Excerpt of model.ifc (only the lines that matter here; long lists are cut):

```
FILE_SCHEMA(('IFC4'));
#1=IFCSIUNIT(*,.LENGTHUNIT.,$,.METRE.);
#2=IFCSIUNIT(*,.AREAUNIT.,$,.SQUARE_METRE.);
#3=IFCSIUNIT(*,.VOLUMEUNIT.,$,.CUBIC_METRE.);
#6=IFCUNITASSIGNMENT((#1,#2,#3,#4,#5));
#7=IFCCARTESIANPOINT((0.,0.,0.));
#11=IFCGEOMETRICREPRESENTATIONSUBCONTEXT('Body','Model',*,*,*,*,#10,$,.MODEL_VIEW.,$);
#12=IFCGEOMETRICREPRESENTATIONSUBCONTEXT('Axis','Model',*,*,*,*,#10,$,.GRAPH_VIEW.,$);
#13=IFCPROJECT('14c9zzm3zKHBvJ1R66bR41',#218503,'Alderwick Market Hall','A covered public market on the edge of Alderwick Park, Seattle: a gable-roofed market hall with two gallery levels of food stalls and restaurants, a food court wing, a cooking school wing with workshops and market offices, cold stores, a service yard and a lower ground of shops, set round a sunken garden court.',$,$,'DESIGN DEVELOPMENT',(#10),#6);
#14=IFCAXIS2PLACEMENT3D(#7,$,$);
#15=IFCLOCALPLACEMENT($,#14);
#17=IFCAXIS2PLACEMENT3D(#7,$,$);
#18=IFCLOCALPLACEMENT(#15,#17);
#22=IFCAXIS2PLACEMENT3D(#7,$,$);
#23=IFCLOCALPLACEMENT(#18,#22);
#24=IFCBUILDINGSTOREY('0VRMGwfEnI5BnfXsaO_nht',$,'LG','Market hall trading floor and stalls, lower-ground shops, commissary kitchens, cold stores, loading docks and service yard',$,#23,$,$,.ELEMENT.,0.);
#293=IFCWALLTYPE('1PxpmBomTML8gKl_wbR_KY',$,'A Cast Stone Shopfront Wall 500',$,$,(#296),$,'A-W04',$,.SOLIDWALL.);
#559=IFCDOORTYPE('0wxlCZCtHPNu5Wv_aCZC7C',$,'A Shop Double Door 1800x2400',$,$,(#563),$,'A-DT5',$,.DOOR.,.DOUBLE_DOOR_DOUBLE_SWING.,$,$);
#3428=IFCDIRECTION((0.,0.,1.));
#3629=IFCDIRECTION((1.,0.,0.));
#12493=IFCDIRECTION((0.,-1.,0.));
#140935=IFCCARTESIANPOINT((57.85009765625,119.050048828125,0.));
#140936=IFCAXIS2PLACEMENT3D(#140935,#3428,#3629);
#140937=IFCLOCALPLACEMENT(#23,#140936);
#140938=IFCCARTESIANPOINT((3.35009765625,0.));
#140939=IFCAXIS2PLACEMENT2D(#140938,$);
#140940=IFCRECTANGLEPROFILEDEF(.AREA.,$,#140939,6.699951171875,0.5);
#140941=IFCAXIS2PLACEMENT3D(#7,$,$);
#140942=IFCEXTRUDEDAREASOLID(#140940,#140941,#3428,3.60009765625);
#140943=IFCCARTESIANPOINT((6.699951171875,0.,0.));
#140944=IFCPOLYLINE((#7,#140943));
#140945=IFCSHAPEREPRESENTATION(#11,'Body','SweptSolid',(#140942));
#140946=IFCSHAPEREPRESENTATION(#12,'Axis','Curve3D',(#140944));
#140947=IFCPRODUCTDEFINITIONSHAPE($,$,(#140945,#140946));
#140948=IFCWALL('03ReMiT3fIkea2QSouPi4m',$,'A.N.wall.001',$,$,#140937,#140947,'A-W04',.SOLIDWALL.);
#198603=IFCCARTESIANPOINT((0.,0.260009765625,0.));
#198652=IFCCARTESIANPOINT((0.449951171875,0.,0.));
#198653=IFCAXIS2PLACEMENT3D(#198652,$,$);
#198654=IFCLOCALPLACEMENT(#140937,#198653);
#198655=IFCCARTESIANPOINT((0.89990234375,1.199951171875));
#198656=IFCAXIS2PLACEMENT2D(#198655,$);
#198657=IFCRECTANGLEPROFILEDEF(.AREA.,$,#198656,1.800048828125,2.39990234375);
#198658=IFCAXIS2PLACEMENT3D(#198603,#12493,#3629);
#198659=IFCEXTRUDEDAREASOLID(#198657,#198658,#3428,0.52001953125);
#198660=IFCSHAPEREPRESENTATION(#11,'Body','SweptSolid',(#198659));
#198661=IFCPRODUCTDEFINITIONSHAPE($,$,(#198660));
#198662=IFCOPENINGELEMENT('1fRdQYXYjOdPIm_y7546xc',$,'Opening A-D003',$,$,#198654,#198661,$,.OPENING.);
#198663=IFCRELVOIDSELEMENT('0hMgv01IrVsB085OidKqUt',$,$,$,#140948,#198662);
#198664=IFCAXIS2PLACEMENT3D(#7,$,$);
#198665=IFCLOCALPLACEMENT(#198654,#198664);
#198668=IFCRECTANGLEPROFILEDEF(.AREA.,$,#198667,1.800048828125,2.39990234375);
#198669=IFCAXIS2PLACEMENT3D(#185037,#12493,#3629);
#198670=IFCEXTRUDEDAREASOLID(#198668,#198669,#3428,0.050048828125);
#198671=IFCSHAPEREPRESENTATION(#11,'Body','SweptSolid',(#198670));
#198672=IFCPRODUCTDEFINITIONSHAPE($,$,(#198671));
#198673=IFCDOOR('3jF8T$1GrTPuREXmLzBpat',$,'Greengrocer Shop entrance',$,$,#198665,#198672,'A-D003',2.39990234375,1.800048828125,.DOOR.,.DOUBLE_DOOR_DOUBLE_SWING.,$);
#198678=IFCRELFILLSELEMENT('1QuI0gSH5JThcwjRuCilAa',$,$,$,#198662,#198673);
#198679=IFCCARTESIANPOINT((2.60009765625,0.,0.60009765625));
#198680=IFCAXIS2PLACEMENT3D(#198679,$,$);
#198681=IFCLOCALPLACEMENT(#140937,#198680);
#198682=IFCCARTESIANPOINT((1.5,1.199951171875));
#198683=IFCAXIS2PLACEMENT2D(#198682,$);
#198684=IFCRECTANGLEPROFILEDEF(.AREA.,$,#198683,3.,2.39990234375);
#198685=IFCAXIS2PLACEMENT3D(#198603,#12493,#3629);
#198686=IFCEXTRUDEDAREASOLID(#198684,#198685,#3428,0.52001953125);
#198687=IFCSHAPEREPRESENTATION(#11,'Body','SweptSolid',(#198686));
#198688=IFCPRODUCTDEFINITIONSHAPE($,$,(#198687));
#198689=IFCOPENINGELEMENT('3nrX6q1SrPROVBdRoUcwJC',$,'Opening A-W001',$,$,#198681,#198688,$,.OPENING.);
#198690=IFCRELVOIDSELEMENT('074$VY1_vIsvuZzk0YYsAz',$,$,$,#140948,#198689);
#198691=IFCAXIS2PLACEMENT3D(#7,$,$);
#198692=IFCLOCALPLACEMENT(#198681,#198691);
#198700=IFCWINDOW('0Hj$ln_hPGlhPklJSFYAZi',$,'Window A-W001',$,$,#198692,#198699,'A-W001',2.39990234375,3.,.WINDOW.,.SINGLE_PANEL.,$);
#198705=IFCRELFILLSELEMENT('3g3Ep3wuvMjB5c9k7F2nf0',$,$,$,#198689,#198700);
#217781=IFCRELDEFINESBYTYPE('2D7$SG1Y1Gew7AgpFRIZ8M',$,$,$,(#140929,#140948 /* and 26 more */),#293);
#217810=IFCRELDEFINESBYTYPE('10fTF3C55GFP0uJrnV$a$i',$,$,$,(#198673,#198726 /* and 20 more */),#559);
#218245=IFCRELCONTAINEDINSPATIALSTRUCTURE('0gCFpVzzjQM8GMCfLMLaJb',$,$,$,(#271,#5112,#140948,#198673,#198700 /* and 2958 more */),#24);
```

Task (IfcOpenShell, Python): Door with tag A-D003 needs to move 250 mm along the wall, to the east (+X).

```python
import ifcopenshell
import ifcopenshell.api.geometry
import ifcopenshell.util.placement

model = ifcopenshell.open("model.ifc")

door = model.by_id(198673)
opening = door.FillsVoids[0].RelatingOpeningElement
wall = opening.VoidsElements[0].RelatingBuildingElement

wall_matrix = ifcopenshell.util.placement.get_local_placement(wall.ObjectPlacement)
shift = wall_matrix[:3, 0] * 0.25
before = ifcopenshell.util.placement.get_local_placement(door.ObjectPlacement)[:3, 3].copy()

# The door is placed relative to its opening, so it follows when the opening moves.
matrix = ifcopenshell.util.placement.get_local_placement(opening.ObjectPlacement)
matrix[:3, 3] += shift
ifcopenshell.api.geometry.edit_object_placement(
    model, product=opening, matrix=matrix, is_si=False, should_transform_children=True
)

after = ifcopenshell.util.placement.get_local_placement(door.ObjectPlacement)[:3, 3]
print("door moved by", (after - before).round(3) + 0.0)

model.write("model-out.ifc")
```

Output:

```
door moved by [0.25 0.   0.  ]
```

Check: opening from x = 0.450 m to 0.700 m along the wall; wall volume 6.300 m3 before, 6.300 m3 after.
